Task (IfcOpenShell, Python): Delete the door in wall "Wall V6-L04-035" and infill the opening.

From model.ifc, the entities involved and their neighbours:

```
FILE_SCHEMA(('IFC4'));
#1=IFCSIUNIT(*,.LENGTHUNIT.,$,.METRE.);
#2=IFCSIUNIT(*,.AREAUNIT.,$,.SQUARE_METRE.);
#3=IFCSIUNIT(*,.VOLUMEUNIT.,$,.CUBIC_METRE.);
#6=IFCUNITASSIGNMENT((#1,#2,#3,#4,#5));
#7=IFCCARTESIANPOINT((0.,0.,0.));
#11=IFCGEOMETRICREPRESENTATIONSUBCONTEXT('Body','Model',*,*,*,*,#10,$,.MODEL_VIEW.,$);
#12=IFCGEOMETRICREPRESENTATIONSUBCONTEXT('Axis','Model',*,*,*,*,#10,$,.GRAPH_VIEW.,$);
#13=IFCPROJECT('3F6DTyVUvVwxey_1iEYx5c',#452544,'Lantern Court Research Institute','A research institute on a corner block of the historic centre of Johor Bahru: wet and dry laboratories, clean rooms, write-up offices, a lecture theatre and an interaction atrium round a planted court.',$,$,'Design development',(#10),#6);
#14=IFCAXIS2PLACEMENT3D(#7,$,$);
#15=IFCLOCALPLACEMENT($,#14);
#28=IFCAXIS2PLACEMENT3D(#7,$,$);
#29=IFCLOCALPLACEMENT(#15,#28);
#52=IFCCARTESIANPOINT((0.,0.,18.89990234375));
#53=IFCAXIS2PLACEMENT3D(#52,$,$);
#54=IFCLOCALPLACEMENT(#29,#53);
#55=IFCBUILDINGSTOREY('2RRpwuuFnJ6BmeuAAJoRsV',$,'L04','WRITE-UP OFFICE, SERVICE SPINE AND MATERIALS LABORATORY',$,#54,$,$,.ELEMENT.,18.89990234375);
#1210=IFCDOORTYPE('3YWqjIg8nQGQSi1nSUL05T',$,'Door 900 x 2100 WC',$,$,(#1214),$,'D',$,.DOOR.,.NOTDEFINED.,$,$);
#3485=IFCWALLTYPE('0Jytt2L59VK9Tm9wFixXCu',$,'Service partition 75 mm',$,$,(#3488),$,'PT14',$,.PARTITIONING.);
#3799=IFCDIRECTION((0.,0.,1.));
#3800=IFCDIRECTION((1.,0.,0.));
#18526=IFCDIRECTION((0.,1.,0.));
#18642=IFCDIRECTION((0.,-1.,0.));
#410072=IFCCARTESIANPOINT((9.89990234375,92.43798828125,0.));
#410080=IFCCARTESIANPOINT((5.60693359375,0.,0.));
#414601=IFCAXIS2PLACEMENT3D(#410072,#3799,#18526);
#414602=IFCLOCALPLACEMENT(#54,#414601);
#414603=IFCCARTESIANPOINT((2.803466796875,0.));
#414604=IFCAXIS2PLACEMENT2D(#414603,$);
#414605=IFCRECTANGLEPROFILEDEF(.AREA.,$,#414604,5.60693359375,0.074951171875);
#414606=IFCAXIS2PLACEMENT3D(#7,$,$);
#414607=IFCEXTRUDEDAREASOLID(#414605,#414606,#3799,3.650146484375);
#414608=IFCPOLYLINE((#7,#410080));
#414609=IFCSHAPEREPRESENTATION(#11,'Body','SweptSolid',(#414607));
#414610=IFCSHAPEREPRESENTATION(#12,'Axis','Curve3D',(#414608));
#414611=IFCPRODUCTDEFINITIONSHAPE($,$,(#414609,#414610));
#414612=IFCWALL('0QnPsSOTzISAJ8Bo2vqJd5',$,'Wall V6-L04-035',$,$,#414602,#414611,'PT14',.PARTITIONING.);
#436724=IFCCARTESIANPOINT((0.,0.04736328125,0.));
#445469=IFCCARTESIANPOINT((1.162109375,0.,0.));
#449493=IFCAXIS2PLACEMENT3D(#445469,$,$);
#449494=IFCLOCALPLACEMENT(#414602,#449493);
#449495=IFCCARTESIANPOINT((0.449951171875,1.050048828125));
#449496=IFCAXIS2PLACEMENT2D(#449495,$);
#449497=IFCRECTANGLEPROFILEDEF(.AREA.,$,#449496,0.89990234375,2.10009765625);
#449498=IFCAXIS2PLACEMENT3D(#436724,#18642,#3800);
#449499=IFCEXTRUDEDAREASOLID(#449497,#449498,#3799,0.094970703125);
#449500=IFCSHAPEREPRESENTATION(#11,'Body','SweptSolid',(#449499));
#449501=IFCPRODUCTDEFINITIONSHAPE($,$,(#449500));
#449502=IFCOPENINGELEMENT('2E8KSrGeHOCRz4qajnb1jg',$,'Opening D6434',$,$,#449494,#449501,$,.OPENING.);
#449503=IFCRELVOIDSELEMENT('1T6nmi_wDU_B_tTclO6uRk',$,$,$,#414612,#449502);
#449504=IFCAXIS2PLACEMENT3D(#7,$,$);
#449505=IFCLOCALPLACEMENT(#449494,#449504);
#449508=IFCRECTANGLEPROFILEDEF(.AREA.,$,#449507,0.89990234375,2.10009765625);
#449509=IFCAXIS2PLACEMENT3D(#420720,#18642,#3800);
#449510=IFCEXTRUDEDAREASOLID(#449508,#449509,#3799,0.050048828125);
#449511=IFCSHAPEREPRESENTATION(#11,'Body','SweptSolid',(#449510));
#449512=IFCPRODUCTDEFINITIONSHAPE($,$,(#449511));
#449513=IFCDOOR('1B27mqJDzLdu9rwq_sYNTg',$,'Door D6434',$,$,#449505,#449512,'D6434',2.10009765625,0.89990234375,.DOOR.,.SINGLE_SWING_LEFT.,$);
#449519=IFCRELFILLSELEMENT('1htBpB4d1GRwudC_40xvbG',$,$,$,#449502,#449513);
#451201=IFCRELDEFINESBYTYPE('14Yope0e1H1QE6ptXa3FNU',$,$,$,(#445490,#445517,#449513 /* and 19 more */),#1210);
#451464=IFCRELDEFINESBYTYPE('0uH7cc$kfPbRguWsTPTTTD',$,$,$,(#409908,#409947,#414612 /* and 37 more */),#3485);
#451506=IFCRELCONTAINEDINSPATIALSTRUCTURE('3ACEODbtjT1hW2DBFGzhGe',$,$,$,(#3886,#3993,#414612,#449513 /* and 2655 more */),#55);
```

```python
import ifcopenshell
import ifcopenshell.api.feature
import ifcopenshell.api.root
import ifcopenshell.geom
import ifcopenshell.util.shape

model = ifcopenshell.open("model.ifc")
settings = ifcopenshell.geom.settings()


def volume(element):
    """Net volume in cubic metres, openings subtracted."""
    shape = ifcopenshell.geom.create_shape(settings, element)
    return ifcopenshell.util.shape.get_volume(shape.geometry)


door = model.by_guid("1B27mqJDzLdu9rwq_sYNTg")
opening = door.FillsVoids[0].RelatingOpeningElement
wall = opening.VoidsElements[0].RelatingBuildingElement
before = volume(wall)

ifcopenshell.api.root.remove_product(model, product=door)
ifcopenshell.api.feature.remove_feature(model, feature=opening)

after = volume(wall)

print(f"wall volume {before:.3f} -> {after:.3f} m3")

model.write("model_v2.ifc")
```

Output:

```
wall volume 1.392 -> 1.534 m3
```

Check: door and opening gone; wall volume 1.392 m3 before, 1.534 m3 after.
